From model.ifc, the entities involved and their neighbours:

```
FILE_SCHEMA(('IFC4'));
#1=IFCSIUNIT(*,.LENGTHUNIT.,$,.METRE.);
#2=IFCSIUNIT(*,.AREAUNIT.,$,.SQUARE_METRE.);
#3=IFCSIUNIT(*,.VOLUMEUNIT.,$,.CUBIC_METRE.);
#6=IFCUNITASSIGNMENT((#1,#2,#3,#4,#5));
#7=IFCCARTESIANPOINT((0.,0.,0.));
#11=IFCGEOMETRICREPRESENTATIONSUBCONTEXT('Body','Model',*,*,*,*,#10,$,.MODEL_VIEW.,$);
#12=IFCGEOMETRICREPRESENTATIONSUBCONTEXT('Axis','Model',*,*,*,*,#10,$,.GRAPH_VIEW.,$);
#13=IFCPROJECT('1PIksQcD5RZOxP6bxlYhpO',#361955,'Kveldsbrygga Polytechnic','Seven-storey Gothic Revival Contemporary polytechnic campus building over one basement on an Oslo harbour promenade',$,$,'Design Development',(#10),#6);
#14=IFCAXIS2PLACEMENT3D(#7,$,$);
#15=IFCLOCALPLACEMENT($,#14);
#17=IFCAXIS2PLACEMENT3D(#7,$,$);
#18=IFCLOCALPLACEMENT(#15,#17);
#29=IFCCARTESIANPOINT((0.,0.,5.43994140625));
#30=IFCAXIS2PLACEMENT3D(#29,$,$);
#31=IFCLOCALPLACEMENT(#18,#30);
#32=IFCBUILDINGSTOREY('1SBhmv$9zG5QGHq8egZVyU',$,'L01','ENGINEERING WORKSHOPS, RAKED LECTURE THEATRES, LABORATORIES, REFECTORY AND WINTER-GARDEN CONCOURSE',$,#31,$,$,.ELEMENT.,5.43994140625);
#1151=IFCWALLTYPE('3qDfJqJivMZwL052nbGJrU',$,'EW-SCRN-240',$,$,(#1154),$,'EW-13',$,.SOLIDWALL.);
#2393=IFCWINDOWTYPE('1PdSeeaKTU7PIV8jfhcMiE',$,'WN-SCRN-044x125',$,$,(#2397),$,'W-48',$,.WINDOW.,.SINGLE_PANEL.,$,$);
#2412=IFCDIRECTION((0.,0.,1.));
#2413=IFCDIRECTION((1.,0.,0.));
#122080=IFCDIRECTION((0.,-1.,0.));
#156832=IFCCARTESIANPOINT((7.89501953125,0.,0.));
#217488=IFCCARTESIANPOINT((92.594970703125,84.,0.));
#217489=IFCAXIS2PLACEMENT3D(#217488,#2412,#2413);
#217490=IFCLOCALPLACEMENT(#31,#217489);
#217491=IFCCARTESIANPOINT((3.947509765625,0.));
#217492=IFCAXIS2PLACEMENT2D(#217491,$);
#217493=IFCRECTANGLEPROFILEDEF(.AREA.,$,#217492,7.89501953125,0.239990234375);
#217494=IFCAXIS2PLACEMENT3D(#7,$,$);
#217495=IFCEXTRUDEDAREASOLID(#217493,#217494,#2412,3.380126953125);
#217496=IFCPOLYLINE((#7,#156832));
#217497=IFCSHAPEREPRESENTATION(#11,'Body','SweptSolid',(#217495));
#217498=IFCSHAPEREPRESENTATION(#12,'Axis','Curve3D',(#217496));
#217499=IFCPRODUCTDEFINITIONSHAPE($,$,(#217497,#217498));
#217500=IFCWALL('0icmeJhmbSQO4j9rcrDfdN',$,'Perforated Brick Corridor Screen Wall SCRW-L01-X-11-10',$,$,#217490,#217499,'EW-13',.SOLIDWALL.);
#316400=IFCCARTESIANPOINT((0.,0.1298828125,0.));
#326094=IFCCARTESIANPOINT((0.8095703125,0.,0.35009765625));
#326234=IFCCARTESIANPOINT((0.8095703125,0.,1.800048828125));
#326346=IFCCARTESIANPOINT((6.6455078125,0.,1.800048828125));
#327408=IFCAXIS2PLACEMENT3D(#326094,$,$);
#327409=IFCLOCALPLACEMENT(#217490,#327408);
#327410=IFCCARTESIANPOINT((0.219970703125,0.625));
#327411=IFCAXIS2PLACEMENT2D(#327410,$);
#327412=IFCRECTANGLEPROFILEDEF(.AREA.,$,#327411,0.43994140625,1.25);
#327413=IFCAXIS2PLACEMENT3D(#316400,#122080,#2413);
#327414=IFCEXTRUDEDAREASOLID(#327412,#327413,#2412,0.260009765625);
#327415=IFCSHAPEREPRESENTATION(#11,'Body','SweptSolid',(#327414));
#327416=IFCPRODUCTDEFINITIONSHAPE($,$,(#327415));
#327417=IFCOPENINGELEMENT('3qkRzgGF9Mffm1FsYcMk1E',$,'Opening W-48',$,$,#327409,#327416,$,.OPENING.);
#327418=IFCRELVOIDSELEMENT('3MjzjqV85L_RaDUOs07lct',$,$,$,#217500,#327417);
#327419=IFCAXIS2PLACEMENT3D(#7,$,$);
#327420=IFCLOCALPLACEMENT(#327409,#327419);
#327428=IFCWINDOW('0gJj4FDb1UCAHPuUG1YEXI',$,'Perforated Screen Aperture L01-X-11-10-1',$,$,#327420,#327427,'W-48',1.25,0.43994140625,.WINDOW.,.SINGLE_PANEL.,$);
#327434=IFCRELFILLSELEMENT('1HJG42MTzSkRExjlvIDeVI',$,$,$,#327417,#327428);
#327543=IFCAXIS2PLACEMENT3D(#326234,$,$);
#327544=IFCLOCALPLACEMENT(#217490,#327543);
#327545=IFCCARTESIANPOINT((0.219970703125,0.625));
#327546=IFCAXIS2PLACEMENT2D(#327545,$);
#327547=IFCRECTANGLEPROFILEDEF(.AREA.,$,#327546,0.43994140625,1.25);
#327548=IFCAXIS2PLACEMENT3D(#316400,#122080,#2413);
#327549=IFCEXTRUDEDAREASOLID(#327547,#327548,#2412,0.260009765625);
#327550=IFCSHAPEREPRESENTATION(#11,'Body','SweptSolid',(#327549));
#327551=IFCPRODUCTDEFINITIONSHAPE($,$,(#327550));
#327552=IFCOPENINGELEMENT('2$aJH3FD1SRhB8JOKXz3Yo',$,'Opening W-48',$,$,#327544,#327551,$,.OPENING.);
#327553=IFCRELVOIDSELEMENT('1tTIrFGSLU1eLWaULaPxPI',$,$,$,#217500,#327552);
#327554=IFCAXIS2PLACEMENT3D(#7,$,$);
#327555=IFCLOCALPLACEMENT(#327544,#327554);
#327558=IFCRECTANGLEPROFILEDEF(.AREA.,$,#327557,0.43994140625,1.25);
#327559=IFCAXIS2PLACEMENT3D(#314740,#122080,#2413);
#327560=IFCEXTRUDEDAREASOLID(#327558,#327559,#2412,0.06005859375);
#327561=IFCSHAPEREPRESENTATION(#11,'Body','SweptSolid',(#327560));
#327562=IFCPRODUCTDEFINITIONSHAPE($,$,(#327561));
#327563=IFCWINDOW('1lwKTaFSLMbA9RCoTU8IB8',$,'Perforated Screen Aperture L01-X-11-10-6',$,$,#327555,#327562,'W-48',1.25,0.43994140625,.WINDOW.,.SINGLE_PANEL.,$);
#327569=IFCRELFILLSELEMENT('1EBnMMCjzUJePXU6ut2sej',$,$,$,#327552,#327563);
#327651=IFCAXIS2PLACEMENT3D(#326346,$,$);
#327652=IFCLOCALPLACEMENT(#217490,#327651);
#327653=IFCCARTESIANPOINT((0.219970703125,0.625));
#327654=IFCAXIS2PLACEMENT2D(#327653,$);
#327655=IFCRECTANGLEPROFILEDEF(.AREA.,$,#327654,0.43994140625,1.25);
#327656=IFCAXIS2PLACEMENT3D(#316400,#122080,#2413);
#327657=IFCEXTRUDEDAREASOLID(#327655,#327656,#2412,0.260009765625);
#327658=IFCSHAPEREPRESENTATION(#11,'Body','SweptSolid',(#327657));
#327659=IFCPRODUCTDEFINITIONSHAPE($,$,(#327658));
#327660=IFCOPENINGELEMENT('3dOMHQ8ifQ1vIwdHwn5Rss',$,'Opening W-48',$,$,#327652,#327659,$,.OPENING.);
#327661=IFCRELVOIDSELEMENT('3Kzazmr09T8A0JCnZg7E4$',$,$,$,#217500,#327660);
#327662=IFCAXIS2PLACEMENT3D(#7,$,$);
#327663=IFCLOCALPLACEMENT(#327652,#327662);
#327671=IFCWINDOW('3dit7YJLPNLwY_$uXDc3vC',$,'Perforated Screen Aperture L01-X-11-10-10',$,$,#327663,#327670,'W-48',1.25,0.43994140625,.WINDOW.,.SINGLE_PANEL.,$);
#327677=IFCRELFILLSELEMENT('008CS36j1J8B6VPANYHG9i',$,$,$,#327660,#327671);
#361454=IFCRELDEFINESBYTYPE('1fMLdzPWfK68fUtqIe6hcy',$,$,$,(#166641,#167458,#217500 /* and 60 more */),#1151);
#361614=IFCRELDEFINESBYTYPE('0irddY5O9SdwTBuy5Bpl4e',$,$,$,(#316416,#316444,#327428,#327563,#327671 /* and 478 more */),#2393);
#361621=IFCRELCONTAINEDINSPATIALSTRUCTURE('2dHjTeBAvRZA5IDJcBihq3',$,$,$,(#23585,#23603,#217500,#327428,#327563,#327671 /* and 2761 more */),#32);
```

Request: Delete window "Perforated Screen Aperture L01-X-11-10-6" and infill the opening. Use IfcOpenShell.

```python
import ifcopenshell
import ifcopenshell.api.feature
import ifcopenshell.api.root
import ifcopenshell.geom
import ifcopenshell.util.shape

model = ifcopenshell.open("model.ifc")
settings = ifcopenshell.geom.settings()


def volume(element):
    """Net volume in cubic metres, openings subtracted."""
    shape = ifcopenshell.geom.create_shape(settings, element)
    return ifcopenshell.util.shape.get_volume(shape.geometry)


window = model.by_guid("1lwKTaFSLMbA9RCoTU8IB8")
opening = window.FillsVoids[0].RelatingOpeningElement
wall = opening.VoidsElements[0].RelatingBuildingElement
before = volume(wall)

ifcopenshell.api.root.remove_product(model, product=window)
ifcopenshell.api.feature.remove_feature(model, feature=opening)

after = volume(wall)

print(f"wall volume {before:.3f} -> {after:.3f} m3")

model.write("model_edited.ifc")
```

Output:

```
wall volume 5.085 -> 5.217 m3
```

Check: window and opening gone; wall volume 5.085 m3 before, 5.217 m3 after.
